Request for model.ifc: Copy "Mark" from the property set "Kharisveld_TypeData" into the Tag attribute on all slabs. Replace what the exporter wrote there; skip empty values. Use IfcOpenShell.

First a look at what the model holds.

```python
import ifcopenshell
import ifcopenshell.util.element

model = ifcopenshell.open("model.ifc")
print(model.schema)
slabs = model.by_type("IfcSlab")
print(len(slabs), "slabs")
for e in slabs[:8]:
    source = ifcopenshell.util.element.get_pset(e, "Kharisveld_TypeData", "Mark")
    target = e.Tag
    print(e.id(), repr(source), repr(target), sep=" | ")
```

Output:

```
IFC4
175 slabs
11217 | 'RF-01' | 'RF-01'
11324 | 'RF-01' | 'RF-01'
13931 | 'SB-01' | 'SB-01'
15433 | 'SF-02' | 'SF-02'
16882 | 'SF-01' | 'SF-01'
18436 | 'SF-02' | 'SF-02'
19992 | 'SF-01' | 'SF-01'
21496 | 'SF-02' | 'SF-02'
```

```python
import ifcopenshell
import ifcopenshell.util.element

model = ifcopenshell.open("model.ifc")

count = 0
for e in model.by_type("IfcSlab"):
    value = ifcopenshell.util.element.get_pset(e, "Kharisveld_TypeData", "Mark")
    current = e.Tag
    if not value or not value.strip() or current == value:
        continue
    e.Tag = value
    count += 1

print(count, "slabs updated")

model.write("model_updated.ifc")
```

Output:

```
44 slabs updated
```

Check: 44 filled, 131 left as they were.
